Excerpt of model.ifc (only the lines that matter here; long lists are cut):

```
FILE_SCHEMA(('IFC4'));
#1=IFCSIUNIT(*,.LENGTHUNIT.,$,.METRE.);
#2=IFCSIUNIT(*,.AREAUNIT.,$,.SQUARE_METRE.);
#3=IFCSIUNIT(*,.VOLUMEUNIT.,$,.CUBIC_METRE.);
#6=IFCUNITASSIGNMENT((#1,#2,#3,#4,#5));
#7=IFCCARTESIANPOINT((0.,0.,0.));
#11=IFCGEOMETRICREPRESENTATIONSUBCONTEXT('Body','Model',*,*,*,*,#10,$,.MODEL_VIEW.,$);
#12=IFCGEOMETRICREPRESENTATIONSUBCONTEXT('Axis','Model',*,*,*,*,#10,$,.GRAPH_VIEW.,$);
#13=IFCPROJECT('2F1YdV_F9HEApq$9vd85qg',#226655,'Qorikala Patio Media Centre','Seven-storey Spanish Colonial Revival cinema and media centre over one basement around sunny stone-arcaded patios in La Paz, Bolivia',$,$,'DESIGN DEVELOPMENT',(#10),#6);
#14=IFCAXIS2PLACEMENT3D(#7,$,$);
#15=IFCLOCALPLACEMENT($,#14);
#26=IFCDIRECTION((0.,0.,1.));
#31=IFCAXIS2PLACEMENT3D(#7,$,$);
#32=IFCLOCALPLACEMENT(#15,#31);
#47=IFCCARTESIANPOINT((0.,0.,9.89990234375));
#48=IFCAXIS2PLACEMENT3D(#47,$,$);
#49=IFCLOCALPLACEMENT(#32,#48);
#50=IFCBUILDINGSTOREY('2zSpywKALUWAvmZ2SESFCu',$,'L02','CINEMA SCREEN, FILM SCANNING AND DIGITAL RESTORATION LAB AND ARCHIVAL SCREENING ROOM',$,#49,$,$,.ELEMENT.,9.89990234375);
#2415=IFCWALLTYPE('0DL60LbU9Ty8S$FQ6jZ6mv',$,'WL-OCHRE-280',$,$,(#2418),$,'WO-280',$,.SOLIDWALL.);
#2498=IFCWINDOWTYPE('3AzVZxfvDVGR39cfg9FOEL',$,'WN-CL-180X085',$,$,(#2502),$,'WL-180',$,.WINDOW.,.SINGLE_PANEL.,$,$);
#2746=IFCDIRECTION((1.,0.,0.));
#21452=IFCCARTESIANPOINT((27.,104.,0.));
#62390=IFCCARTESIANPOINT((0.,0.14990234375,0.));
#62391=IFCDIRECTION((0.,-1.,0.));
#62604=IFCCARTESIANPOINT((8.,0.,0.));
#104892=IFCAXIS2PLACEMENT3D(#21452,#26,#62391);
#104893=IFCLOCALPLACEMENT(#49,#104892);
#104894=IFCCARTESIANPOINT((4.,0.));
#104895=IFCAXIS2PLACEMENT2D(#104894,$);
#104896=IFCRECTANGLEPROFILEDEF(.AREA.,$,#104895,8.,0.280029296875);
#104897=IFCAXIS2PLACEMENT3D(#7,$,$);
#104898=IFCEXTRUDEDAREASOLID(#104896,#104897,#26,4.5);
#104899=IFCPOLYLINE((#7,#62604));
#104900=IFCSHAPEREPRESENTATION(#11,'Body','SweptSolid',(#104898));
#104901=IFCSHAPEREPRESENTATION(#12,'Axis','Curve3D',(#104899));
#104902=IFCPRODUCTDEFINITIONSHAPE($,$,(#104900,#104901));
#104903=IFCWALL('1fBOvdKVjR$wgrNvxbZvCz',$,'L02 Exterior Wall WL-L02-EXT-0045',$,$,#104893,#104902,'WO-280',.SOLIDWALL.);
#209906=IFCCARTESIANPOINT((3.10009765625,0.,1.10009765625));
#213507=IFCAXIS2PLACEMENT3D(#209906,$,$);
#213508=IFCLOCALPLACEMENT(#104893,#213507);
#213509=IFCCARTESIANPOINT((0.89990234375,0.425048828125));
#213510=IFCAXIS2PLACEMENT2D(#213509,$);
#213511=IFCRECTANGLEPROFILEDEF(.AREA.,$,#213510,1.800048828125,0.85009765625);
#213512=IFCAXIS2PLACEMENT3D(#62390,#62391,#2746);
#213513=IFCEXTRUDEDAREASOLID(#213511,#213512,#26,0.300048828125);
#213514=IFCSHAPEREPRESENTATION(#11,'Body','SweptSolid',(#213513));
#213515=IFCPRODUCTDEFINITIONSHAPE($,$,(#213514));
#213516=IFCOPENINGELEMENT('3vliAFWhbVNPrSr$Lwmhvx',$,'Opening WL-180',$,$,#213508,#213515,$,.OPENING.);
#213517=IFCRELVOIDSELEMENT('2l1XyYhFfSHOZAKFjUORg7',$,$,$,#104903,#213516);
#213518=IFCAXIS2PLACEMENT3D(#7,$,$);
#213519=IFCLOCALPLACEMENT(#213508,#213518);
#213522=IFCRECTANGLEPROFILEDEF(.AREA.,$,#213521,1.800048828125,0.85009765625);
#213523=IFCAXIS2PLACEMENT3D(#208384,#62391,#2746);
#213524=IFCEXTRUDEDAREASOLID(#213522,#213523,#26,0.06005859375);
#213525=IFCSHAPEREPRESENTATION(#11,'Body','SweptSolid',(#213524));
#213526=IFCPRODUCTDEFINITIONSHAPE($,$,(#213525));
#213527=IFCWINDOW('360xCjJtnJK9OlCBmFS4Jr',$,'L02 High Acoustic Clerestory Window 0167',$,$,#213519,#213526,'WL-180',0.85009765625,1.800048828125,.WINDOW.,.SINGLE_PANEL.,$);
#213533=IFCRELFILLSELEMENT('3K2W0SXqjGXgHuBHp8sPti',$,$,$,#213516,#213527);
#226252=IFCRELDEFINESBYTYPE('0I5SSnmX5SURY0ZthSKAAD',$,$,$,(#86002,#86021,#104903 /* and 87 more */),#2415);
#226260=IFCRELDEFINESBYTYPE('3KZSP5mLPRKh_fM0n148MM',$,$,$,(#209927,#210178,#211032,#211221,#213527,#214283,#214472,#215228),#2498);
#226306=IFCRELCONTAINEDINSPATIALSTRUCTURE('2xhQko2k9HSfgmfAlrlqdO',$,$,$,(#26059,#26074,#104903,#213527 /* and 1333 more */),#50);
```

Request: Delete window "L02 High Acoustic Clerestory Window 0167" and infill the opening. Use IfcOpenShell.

```python
import ifcopenshell
import ifcopenshell.api.feature
import ifcopenshell.api.root
import ifcopenshell.geom
import ifcopenshell.util.shape

model = ifcopenshell.open("model.ifc")
settings = ifcopenshell.geom.settings()


def volume(element):
    """Net volume in cubic metres, openings subtracted."""
    shape = ifcopenshell.geom.create_shape(settings, element)
    return ifcopenshell.util.shape.get_volume(shape.geometry)


window = model.by_guid("360xCjJtnJK9OlCBmFS4Jr")
opening = window.FillsVoids[0].RelatingOpeningElement
wall = opening.VoidsElements[0].RelatingBuildingElement
before = volume(wall)

ifcopenshell.api.root.remove_product(model, product=window)
ifcopenshell.api.feature.remove_feature(model, feature=opening)

after = volume(wall)

print(f"wall volume {before:.3f} -> {after:.3f} m3")

model.write("model_v2.ifc")
```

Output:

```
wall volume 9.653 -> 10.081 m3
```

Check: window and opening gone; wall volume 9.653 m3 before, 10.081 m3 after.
